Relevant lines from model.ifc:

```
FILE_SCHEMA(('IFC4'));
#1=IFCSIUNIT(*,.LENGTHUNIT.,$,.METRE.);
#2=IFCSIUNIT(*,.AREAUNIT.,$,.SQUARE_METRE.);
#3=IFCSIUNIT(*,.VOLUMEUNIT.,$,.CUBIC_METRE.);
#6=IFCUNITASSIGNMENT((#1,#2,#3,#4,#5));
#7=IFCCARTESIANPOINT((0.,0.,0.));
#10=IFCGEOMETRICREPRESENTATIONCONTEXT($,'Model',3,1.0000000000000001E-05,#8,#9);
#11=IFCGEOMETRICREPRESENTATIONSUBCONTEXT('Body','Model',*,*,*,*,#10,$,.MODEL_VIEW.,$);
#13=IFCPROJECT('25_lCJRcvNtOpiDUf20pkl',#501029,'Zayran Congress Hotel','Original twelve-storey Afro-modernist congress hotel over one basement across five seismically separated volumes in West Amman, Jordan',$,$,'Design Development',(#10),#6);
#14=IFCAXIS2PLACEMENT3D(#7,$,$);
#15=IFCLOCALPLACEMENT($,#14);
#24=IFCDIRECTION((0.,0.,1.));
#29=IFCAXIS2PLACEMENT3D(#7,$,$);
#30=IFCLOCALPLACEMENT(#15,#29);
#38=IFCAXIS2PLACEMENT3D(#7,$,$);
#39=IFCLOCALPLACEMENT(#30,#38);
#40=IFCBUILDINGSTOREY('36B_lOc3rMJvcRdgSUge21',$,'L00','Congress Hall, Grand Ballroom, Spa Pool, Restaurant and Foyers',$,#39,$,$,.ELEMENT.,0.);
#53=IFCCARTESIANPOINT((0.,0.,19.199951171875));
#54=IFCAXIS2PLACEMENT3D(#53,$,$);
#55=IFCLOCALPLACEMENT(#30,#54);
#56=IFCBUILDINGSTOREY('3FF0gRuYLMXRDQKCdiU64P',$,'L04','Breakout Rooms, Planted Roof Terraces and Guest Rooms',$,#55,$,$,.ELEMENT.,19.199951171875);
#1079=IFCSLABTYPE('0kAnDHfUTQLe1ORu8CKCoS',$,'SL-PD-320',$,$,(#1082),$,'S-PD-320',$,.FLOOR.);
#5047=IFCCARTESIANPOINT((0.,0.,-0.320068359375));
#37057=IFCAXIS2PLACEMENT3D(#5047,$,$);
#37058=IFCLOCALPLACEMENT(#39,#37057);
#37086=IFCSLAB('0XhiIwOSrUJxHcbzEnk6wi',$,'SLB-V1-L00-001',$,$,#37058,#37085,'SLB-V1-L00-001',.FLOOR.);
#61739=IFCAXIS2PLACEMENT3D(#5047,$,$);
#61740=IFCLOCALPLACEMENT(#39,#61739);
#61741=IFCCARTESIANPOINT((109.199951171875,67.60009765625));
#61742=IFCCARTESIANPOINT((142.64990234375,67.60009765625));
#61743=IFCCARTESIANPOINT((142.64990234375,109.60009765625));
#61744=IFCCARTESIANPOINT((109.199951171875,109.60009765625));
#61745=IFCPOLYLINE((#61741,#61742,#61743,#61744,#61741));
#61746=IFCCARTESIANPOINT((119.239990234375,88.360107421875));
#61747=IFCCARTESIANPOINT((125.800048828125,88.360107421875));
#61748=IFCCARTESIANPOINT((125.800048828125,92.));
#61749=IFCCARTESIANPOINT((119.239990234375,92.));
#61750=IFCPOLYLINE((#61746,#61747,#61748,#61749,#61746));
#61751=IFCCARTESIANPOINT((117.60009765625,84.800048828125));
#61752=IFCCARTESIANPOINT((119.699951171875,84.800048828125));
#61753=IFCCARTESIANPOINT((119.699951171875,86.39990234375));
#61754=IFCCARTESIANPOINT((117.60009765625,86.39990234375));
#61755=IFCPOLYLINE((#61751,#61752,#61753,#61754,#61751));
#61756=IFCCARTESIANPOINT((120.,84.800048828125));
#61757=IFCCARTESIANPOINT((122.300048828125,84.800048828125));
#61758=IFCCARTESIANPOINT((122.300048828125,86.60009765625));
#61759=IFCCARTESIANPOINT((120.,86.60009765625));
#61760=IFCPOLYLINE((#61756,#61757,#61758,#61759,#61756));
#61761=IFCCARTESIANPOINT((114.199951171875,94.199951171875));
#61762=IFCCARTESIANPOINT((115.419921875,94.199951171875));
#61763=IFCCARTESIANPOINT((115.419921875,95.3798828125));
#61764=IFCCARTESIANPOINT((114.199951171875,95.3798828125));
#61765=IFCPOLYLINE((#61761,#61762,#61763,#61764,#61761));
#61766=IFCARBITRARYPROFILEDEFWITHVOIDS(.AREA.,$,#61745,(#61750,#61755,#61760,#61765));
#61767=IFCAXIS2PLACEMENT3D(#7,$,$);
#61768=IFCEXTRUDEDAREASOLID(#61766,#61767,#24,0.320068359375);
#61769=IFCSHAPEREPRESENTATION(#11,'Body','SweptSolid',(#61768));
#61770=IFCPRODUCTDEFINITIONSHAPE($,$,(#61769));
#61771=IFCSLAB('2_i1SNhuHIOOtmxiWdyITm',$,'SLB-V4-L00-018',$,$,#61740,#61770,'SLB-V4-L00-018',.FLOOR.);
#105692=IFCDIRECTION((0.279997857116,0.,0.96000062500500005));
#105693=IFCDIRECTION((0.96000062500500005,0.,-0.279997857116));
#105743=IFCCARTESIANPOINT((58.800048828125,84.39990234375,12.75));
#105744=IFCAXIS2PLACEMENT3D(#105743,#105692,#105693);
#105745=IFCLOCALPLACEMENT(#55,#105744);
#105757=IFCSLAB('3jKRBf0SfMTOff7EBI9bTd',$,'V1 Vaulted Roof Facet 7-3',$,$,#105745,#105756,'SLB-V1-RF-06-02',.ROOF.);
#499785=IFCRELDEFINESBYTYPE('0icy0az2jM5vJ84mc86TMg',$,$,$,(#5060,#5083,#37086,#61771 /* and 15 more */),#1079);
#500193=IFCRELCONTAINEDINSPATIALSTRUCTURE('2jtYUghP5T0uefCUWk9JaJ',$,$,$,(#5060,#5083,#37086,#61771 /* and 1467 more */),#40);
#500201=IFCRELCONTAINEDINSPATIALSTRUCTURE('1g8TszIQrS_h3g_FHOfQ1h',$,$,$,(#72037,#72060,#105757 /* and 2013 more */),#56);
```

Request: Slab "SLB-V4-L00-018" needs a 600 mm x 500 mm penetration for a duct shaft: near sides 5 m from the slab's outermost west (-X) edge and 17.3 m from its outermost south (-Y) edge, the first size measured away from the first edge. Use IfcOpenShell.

```python
import numpy as np
import ifcopenshell
import ifcopenshell.api.feature
import ifcopenshell.api.geometry
import ifcopenshell.api.root
import ifcopenshell.geom
import ifcopenshell.util.placement
import ifcopenshell.util.representation
import ifcopenshell.util.shape
import ifcopenshell.util.unit

model = ifcopenshell.open("model.ifc")
unit_scale = ifcopenshell.util.unit.calculate_unit_scale(model)
settings = ifcopenshell.geom.settings()


def volume(element):
    """Net volume in cubic metres, openings subtracted."""
    shape = ifcopenshell.geom.create_shape(settings, element)
    return ifcopenshell.util.shape.get_volume(shape.geometry)


slab = model.by_guid("2_i1SNhuHIOOtmxiWdyITm")
before = volume(slab)

# Extent in the slab's own axes, in metres. The edges named are its -X and -Y sides.
slab_shape = ifcopenshell.geom.create_shape(settings, slab)
vertices = ifcopenshell.util.shape.get_vertices(slab_shape.geometry)
x_min, y_min, bottom = vertices.min(axis=0)
top = vertices[:, 2].max()

opening = ifcopenshell.api.root.create_entity(model, ifc_class="IfcOpeningElement", name="Duct shaft opening", predefined_type="OPENING")
context = ifcopenshell.util.representation.get_context(model, "Model", "Body", "MODEL_VIEW")
width, depth = 0.6, 0.5
outline = [(0.0, 0.0), (width, 0.0), (width, depth), (0.0, depth), (0.0, 0.0)]
# Overshoot both faces by 50 mm so the cut is clean.
shape = ifcopenshell.api.geometry.add_slab_representation(
    model, context=context, depth=top - bottom + 0.1, polyline=outline
)
ifcopenshell.api.geometry.assign_representation(model, product=opening, representation=shape)

matrix = ifcopenshell.util.placement.get_local_placement(slab.ObjectPlacement)
matrix[:, 3] = matrix @ np.append(np.array([x_min + 5, y_min + 17.3, bottom - 0.05]) / unit_scale, 1.0)
ifcopenshell.api.geometry.edit_object_placement(model, product=opening, matrix=matrix, is_si=False)
ifcopenshell.api.feature.add_feature(model, feature=opening, element=slab)

after = volume(slab)

print(f"slab volume {before:.3f} -> {after:.3f} m3")

model.write("model_v2.ifc")
```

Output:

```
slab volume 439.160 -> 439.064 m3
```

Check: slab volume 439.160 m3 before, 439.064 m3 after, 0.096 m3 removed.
